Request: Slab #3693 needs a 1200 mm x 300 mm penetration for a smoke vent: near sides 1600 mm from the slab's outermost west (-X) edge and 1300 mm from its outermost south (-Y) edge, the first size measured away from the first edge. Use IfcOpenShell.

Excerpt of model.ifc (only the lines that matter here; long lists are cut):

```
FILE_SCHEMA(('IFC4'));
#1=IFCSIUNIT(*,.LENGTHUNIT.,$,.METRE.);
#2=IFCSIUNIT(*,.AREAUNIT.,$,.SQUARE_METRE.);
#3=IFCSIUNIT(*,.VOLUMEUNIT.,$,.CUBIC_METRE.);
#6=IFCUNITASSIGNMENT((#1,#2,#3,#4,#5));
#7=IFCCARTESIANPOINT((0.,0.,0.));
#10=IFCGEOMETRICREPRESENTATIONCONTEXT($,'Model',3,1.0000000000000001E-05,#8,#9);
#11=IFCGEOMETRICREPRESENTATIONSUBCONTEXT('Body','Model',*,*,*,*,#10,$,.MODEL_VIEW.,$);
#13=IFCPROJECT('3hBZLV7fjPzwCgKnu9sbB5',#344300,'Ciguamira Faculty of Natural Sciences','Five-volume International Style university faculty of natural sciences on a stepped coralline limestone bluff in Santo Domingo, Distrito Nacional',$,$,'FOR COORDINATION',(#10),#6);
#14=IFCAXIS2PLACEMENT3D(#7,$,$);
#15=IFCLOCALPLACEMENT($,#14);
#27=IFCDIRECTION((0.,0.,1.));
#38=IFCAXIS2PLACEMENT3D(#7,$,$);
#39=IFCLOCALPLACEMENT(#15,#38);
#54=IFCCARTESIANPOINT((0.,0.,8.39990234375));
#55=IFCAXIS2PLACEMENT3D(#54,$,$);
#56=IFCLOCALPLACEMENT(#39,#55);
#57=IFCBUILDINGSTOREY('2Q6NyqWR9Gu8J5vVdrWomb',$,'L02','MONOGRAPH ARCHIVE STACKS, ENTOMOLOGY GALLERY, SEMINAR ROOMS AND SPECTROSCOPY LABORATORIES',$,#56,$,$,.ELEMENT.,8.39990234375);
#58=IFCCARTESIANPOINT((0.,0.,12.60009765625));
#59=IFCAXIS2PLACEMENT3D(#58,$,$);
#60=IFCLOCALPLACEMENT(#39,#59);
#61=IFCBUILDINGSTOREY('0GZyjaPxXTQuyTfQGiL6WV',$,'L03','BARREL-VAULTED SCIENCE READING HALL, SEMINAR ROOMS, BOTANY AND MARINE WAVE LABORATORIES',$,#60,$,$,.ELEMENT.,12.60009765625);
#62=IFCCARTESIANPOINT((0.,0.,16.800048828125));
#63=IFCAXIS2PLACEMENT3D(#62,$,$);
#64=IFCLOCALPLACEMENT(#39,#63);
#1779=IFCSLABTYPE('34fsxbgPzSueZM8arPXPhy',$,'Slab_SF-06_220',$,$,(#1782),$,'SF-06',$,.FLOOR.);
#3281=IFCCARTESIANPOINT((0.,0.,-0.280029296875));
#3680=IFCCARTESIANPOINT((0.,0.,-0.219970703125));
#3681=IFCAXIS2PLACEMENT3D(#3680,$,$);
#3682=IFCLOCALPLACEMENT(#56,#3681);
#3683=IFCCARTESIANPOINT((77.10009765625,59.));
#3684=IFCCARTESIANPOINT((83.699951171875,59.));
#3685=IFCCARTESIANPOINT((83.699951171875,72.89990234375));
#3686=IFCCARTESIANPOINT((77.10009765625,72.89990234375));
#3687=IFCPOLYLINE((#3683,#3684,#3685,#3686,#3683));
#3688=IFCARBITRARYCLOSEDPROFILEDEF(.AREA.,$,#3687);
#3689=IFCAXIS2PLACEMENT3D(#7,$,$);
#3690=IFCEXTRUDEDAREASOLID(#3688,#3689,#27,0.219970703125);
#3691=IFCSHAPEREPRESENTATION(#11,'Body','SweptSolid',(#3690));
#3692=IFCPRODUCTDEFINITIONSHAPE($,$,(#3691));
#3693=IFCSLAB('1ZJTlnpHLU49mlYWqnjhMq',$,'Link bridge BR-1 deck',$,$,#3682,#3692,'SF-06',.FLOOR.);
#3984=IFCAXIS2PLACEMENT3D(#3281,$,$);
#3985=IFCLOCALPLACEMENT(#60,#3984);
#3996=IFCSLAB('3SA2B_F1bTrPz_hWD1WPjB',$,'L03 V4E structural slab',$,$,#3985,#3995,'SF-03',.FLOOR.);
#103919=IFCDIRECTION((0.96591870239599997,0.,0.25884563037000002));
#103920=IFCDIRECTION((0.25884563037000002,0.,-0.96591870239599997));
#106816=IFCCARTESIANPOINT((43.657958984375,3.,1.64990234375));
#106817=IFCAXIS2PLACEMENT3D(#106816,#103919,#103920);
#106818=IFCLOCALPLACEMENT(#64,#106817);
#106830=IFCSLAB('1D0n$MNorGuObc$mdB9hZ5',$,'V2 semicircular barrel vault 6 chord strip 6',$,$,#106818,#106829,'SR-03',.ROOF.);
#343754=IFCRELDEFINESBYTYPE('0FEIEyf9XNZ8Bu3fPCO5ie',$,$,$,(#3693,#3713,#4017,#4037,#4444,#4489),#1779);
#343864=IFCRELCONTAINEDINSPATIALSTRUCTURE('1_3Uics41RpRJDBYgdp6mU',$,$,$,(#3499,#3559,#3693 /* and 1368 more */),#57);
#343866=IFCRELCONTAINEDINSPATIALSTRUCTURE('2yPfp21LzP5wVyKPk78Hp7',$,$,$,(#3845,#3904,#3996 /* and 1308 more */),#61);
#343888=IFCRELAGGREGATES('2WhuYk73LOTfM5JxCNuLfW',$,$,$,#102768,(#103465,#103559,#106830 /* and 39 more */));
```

```python
import numpy as np
import ifcopenshell
import ifcopenshell.api.feature
import ifcopenshell.api.geometry
import ifcopenshell.api.root
import ifcopenshell.geom
import ifcopenshell.util.placement
import ifcopenshell.util.representation
import ifcopenshell.util.shape
import ifcopenshell.util.unit

model = ifcopenshell.open("model.ifc")
unit_scale = ifcopenshell.util.unit.calculate_unit_scale(model)
settings = ifcopenshell.geom.settings()


def volume(element):
    """Net volume in cubic metres, openings subtracted."""
    shape = ifcopenshell.geom.create_shape(settings, element)
    return ifcopenshell.util.shape.get_volume(shape.geometry)


slab = model.by_guid("1ZJTlnpHLU49mlYWqnjhMq")
before = volume(slab)

# Extent in the slab's own axes, in metres. The edges named are its -X and -Y sides.
slab_shape = ifcopenshell.geom.create_shape(settings, slab)
vertices = ifcopenshell.util.shape.get_vertices(slab_shape.geometry)
x_min, y_min, bottom = vertices.min(axis=0)
top = vertices[:, 2].max()

opening = ifcopenshell.api.root.create_entity(model, ifc_class="IfcOpeningElement", name="Smoke vent opening", predefined_type="OPENING")
context = ifcopenshell.util.representation.get_context(model, "Model", "Body", "MODEL_VIEW")
width, depth = 1.2, 0.3
outline = [(0.0, 0.0), (width, 0.0), (width, depth), (0.0, depth), (0.0, 0.0)]
# Overshoot both faces by 50 mm so the cut is clean.
shape = ifcopenshell.api.geometry.add_slab_representation(
    model, context=context, depth=top - bottom + 0.1, polyline=outline
)
ifcopenshell.api.geometry.assign_representation(model, product=opening, representation=shape)

matrix = ifcopenshell.util.placement.get_local_placement(slab.ObjectPlacement)
matrix[:, 3] = matrix @ np.append(np.array([x_min + 1.6, y_min + 1.3, bottom - 0.05]) / unit_scale, 1.0)
ifcopenshell.api.geometry.edit_object_placement(model, product=opening, matrix=matrix, is_si=False)
ifcopenshell.api.feature.add_feature(model, feature=opening, element=slab)

after = volume(slab)

print(f"slab volume {before:.3f} -> {after:.3f} m3")

model.write("model-out.ifc")
```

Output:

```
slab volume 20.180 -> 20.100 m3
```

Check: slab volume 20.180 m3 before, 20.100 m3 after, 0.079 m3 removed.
